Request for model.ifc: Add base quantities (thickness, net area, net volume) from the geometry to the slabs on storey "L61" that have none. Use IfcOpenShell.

First a look at what the model holds.

```python
import ifcopenshell
import ifcopenshell.util.element
import ifcopenshell.util.unit

model = ifcopenshell.open("model.ifc")
print(model.schema)
for unit_type in ("LENGTHUNIT", "AREAUNIT", "VOLUMEUNIT"):
    print(unit_type, ifcopenshell.util.unit.calculate_unit_scale(model, unit_type))
storey = next(s for s in model.by_type("IfcBuildingStorey") if s.Name == "L61")
slabs = [e for e in ifcopenshell.util.element.get_decomposition(storey) if e.is_a("IfcSlab")]
for e in sorted(slabs, key=lambda e: e.id()):
    print(e.id(), e.is_a(), e.Name, list(ifcopenshell.util.element.get_psets(e, qtos_only=True)), sep=" | ")
```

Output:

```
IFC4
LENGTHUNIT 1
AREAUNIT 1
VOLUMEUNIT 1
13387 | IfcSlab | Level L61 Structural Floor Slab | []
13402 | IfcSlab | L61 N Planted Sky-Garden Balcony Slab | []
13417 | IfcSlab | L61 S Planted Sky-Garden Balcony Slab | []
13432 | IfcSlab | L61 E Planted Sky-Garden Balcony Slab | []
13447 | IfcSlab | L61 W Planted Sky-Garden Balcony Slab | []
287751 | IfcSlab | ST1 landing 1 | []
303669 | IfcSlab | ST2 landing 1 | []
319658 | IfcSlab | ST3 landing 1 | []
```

```python
import ifcopenshell
import ifcopenshell.api.pset
import ifcopenshell.geom
import ifcopenshell.util.element
import ifcopenshell.util.shape
import ifcopenshell.util.unit

model = ifcopenshell.open("model.ifc")
unit_scale = ifcopenshell.util.unit.calculate_unit_scale(model)
area_scale = ifcopenshell.util.unit.calculate_unit_scale(model, "AREAUNIT")
volume_scale = ifcopenshell.util.unit.calculate_unit_scale(model, "VOLUMEUNIT")
settings = ifcopenshell.geom.settings()

storey = next(s for s in model.by_type("IfcBuildingStorey") if s.Name == "L61")
slabs = [e for e in ifcopenshell.util.element.get_decomposition(storey) if e.is_a("IfcSlab")]

for e in sorted(slabs, key=lambda e: e.id()):
    if ifcopenshell.util.element.get_psets(e, qtos_only=True, should_inherit=False):
        continue
    # Geometry comes back in metres, in the element's own axes.
    shape = ifcopenshell.geom.create_shape(settings, e)
    values = {
        "Width": ifcopenshell.util.shape.get_z(shape.geometry) / unit_scale,
        "NetArea": ifcopenshell.util.shape.get_footprint_area(shape.geometry) / area_scale,
        "NetVolume": ifcopenshell.util.shape.get_volume(shape.geometry) / volume_scale,
    }
    qto = ifcopenshell.api.pset.add_qto(model, product=e, name="Qto_SlabBaseQuantities")
    ifcopenshell.api.pset.edit_qto(model, qto=qto, properties=values)
    print(e.id(), {k: round(v, 3) for k, v in values.items()})

model.write("model_edited.ifc")
```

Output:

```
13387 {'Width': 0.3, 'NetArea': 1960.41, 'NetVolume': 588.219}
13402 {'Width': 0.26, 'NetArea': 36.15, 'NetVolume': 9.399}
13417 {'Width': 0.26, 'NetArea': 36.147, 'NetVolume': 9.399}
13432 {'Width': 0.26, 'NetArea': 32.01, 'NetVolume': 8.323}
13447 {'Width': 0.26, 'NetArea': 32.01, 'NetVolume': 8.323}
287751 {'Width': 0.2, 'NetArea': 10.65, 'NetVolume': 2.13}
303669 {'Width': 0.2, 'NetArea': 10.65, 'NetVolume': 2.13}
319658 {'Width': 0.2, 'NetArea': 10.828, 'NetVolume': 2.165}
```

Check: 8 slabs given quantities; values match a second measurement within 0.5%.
